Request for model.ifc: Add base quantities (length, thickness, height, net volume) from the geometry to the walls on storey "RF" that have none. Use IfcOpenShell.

First a look at what the model holds.

```python
import ifcopenshell
import ifcopenshell.util.element
import ifcopenshell.util.unit

model = ifcopenshell.open("model.ifc")
print(model.schema)
for unit_type in ("LENGTHUNIT", "AREAUNIT", "VOLUMEUNIT"):
    print(unit_type, ifcopenshell.util.unit.calculate_unit_scale(model, unit_type))
storey = next(s for s in model.by_type("IfcBuildingStorey") if s.Name == "RF")
walls = [e for e in ifcopenshell.util.element.get_decomposition(storey) if e.is_a("IfcWall")]
for e in sorted(walls, key=lambda e: e.id()):
    print(e.id(), e.is_a(), e.Name, list(ifcopenshell.util.element.get_psets(e, qtos_only=True)), sep=" | ")
```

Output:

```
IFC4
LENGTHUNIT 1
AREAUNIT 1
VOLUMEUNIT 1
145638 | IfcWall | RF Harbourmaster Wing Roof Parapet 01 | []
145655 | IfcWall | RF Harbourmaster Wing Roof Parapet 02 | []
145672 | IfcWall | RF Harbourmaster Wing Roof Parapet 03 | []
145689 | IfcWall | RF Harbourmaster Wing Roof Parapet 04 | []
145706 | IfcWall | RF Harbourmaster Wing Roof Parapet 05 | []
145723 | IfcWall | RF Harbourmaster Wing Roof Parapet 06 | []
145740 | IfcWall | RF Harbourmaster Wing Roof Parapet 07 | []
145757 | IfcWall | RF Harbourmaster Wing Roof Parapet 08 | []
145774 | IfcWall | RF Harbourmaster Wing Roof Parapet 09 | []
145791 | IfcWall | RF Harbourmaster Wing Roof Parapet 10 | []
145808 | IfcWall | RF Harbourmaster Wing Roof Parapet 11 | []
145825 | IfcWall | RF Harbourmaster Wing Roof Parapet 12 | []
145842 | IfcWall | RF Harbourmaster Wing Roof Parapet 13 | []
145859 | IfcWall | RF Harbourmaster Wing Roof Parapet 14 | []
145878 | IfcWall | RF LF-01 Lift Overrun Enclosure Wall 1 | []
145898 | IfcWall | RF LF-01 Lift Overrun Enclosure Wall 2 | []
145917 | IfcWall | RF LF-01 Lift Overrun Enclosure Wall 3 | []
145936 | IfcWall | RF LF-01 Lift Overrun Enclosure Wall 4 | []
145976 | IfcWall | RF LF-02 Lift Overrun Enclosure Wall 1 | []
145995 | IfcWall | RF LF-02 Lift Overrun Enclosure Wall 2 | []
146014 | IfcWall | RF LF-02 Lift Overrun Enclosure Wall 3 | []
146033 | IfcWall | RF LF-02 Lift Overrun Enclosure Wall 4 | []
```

```python
import ifcopenshell
import ifcopenshell.api.pset
import ifcopenshell.geom
import ifcopenshell.util.element
import ifcopenshell.util.shape
import ifcopenshell.util.unit

model = ifcopenshell.open("model.ifc")
unit_scale = ifcopenshell.util.unit.calculate_unit_scale(model)
volume_scale = ifcopenshell.util.unit.calculate_unit_scale(model, "VOLUMEUNIT")
settings = ifcopenshell.geom.settings()

storey = next(s for s in model.by_type("IfcBuildingStorey") if s.Name == "RF")
walls = [e for e in ifcopenshell.util.element.get_decomposition(storey) if e.is_a("IfcWall")]

for e in sorted(walls, key=lambda e: e.id()):
    if ifcopenshell.util.element.get_psets(e, qtos_only=True, should_inherit=False):
        continue
    # Geometry comes back in metres, in the element's own axes.
    shape = ifcopenshell.geom.create_shape(settings, e)
    values = {
        "Length": ifcopenshell.util.shape.get_x(shape.geometry) / unit_scale,
        "Width": ifcopenshell.util.shape.get_y(shape.geometry) / unit_scale,
        "Height": ifcopenshell.util.shape.get_z(shape.geometry) / unit_scale,
        "NetVolume": ifcopenshell.util.shape.get_volume(shape.geometry) / volume_scale,
    }
    qto = ifcopenshell.api.pset.add_qto(model, product=e, name="Qto_WallBaseQuantities")
    ifcopenshell.api.pset.edit_qto(model, qto=qto, properties=values)
    print(e.id(), {k: round(v, 3) for k, v in values.items()})

model.write("model_v2.ifc")
```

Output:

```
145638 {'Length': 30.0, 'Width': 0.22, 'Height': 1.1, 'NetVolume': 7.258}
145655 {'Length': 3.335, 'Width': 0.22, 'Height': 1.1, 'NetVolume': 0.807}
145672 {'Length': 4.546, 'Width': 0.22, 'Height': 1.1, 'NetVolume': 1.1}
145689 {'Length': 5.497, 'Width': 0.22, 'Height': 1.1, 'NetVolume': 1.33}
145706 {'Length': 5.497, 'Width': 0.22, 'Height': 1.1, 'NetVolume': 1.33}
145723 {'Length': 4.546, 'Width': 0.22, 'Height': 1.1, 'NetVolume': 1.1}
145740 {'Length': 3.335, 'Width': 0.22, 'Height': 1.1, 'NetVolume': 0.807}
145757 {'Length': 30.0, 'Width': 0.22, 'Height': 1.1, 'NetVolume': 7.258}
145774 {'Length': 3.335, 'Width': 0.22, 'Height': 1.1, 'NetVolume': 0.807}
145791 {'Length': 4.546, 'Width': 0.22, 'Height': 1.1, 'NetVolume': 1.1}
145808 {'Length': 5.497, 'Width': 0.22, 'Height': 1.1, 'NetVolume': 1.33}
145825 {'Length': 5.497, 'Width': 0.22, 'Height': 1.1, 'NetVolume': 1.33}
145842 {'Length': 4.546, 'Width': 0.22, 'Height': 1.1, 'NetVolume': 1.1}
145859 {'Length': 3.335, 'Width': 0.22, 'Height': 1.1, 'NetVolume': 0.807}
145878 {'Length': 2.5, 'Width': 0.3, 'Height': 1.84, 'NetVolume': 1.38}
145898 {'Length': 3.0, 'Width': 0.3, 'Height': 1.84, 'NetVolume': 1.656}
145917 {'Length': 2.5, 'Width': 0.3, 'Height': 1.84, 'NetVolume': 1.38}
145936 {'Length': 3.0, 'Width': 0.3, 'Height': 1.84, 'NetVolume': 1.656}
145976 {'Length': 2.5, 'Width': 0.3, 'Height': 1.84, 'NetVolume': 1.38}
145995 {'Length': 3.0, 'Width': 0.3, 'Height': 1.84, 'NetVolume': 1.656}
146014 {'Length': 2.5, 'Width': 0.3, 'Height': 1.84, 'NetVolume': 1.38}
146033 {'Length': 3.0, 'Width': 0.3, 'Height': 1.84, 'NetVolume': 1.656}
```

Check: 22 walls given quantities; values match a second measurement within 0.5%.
